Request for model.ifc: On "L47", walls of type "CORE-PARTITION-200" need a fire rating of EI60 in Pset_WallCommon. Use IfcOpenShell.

First a look at what the model holds.

```python
import ifcopenshell
import ifcopenshell.util.element

model = ifcopenshell.open("model.ifc")
print(model.schema)
storey = next(s for s in model.by_type("IfcBuildingStorey") if s.Name == "L47")
walls = [e for e in ifcopenshell.util.element.get_decomposition(storey) if e.is_a("IfcWall")]
seen = {}
for e in walls:
    element_type = ifcopenshell.util.element.get_type(e)
    key = (element_type.Name if element_type != e and element_type else None, ifcopenshell.util.element.get_pset(e, "Pset_WallCommon", "FireRating"))
    seen[key] = seen.get(key, 0) + 1
for (name, value), count in sorted(seen.items(), key=str):
    print(count, "x", name, "|", value)
```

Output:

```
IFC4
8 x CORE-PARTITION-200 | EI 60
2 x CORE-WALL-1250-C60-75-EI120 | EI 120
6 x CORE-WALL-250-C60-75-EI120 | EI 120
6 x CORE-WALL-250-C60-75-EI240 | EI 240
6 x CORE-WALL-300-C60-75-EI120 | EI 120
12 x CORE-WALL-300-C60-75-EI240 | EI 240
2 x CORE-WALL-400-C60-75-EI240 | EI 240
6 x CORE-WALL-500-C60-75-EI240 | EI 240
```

```python
import ifcopenshell
import ifcopenshell.api.pset
import ifcopenshell.util.element

model = ifcopenshell.open("model.ifc")

storey = next(s for s in model.by_type("IfcBuildingStorey") if s.Name == "L47")
walls = [e for e in ifcopenshell.util.element.get_decomposition(storey) if e.is_a("IfcWall")]

count = 0
for e in walls:
    element_type = ifcopenshell.util.element.get_type(e)
    if element_type in (None, e) or element_type.Name != "CORE-PARTITION-200":
        continue
    found = ifcopenshell.util.element.get_pset(e, "Pset_WallCommon", should_inherit=False)
    if found:
        pset = model.by_id(found["id"])
        if len(ifcopenshell.util.element.get_elements_by_pset(pset)) > 1:
            pset = ifcopenshell.api.pset.unshare_pset(model, products=[e], pset=pset)[0]
    else:
        pset = ifcopenshell.api.pset.add_pset(model, product=e, name="Pset_WallCommon")
    ifcopenshell.api.pset.edit_pset(model, pset=pset, properties={"FireRating": "EI60"})
    count += 1

print(count, "walls updated")

model.write("model_rev.ifc")
```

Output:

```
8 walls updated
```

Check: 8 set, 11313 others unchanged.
